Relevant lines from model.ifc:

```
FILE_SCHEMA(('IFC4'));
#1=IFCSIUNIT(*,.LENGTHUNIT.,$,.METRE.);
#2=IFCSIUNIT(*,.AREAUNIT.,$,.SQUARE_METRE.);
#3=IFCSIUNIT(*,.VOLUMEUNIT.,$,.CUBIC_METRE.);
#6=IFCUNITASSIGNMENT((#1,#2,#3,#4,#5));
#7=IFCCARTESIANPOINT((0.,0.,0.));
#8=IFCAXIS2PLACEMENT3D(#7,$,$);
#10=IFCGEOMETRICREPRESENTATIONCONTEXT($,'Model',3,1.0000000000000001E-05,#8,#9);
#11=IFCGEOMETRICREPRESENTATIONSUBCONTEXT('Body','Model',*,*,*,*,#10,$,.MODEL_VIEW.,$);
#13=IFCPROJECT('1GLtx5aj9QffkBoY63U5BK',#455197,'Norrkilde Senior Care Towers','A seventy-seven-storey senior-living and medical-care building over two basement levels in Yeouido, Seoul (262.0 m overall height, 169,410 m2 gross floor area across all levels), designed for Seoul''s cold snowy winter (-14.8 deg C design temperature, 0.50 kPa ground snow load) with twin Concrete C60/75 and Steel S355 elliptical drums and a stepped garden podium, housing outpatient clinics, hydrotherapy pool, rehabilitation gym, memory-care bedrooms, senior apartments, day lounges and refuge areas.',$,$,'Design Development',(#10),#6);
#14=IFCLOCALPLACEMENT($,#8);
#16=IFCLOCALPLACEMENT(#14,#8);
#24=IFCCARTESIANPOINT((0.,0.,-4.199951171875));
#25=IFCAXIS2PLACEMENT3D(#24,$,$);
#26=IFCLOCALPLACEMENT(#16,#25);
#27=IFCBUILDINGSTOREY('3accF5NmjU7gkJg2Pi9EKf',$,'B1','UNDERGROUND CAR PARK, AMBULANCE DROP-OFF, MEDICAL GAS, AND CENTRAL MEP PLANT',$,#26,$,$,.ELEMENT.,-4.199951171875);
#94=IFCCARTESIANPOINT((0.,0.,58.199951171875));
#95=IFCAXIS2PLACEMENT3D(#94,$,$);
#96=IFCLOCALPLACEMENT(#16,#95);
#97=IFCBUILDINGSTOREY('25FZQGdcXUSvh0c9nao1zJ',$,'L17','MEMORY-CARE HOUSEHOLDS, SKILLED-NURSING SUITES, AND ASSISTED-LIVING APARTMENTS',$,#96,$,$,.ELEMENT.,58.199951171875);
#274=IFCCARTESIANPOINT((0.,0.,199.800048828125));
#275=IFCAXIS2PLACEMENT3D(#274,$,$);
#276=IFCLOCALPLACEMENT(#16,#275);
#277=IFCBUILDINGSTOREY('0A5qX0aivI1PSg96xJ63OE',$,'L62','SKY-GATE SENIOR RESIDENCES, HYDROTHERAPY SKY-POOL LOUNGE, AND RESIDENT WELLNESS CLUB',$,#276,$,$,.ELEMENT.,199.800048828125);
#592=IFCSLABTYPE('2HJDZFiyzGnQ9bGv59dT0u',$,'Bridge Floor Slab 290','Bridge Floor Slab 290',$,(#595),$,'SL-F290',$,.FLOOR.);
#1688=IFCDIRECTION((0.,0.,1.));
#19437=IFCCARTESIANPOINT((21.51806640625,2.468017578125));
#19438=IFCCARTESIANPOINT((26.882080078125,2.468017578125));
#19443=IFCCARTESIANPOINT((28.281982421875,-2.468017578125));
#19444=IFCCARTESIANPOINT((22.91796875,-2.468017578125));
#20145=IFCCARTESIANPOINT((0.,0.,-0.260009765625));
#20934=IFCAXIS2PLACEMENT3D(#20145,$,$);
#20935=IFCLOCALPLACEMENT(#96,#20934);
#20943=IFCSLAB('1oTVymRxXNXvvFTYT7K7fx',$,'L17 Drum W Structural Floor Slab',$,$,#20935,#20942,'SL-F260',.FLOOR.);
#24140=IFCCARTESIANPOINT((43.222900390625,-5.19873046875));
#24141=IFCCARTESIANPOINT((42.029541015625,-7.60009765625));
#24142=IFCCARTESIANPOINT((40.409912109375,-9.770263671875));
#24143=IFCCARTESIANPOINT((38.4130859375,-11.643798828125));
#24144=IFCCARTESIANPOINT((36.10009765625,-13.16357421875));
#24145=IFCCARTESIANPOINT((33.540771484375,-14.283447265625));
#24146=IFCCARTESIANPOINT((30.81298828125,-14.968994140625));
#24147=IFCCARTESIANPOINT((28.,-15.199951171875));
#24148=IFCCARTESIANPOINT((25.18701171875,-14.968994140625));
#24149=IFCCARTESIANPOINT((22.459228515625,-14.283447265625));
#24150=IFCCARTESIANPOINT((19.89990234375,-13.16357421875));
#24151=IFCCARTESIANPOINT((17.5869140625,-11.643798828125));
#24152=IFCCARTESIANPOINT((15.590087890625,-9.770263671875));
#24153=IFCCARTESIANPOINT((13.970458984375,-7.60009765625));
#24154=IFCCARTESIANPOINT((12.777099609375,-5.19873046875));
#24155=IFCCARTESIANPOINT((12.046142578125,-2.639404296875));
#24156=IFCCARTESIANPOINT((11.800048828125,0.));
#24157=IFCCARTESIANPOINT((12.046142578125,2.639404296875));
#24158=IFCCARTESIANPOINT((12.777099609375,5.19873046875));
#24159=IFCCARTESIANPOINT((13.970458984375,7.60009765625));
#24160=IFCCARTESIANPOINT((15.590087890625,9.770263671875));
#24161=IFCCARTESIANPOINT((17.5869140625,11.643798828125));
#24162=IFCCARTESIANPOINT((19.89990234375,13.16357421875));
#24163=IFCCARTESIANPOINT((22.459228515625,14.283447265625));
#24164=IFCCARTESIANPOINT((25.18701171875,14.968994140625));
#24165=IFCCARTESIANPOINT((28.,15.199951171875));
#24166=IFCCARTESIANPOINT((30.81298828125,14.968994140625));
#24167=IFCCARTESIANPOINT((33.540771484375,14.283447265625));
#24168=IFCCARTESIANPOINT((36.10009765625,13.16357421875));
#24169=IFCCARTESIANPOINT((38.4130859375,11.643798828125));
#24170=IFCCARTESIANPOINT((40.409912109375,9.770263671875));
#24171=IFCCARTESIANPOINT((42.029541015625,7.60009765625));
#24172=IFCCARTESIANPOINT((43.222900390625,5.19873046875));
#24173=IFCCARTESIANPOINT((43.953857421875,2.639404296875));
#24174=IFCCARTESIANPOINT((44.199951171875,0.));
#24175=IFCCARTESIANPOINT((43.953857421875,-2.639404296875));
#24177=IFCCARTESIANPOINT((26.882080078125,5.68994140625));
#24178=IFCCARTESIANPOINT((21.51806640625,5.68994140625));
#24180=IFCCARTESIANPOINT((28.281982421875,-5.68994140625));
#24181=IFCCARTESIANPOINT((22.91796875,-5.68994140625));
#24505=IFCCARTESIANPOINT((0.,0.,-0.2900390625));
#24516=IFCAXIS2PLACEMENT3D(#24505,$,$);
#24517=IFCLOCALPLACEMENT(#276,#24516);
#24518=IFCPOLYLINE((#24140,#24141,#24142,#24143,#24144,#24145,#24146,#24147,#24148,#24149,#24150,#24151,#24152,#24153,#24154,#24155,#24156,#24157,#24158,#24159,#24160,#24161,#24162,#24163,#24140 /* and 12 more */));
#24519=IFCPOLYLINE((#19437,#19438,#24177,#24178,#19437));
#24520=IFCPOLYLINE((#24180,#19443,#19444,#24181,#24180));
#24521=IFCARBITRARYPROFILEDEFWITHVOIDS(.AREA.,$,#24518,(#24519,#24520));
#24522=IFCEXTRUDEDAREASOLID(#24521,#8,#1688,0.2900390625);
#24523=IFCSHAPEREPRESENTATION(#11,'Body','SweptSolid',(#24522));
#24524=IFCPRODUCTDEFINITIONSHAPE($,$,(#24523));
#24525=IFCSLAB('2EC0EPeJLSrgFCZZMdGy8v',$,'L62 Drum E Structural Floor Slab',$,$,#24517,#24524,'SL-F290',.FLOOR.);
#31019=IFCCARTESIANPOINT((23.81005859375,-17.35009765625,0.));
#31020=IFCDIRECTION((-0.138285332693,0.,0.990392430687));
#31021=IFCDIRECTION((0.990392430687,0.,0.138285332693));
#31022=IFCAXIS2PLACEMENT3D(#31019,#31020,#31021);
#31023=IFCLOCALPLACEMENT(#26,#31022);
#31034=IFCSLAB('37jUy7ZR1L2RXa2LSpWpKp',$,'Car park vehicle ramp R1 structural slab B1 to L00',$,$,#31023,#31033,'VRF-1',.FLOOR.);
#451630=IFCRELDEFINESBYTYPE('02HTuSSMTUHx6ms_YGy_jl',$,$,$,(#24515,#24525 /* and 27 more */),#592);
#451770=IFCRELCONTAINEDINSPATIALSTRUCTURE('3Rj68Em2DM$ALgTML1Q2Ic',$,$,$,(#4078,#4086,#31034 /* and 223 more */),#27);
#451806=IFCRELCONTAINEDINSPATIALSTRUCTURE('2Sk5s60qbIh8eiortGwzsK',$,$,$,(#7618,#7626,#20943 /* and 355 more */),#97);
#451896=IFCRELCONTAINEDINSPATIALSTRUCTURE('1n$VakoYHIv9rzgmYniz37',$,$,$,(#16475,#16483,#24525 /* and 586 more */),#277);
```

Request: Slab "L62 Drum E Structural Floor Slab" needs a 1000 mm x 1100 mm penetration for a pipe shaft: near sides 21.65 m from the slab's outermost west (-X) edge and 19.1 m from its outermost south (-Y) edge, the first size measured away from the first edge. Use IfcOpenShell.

```python
import numpy as np
import ifcopenshell
import ifcopenshell.api.feature
import ifcopenshell.api.geometry
import ifcopenshell.api.root
import ifcopenshell.geom
import ifcopenshell.util.placement
import ifcopenshell.util.representation
import ifcopenshell.util.shape
import ifcopenshell.util.unit

model = ifcopenshell.open("model.ifc")
unit_scale = ifcopenshell.util.unit.calculate_unit_scale(model)
settings = ifcopenshell.geom.settings()


def volume(element):
    """Net volume in cubic metres, openings subtracted."""
    shape = ifcopenshell.geom.create_shape(settings, element)
    return ifcopenshell.util.shape.get_volume(shape.geometry)


slab = model.by_guid("2EC0EPeJLSrgFCZZMdGy8v")
before = volume(slab)

# Extent in the slab's own axes, in metres. The edges named are its -X and -Y sides.
slab_shape = ifcopenshell.geom.create_shape(settings, slab)
vertices = ifcopenshell.util.shape.get_vertices(slab_shape.geometry)
x_min, y_min, bottom = vertices.min(axis=0)
top = vertices[:, 2].max()

opening = ifcopenshell.api.root.create_entity(model, ifc_class="IfcOpeningElement", name="Pipe shaft opening", predefined_type="OPENING")
context = ifcopenshell.util.representation.get_context(model, "Model", "Body", "MODEL_VIEW")
width, depth = 1, 1.1
outline = [(0.0, 0.0), (width, 0.0), (width, depth), (0.0, depth), (0.0, 0.0)]
# Overshoot both faces by 50 mm so the cut is clean.
shape = ifcopenshell.api.geometry.add_slab_representation(
    model, context=context, depth=top - bottom + 0.1, polyline=outline
)
ifcopenshell.api.geometry.assign_representation(model, product=opening, representation=shape)

matrix = ifcopenshell.util.placement.get_local_placement(slab.ObjectPlacement)
matrix[:, 3] = matrix @ np.append(np.array([x_min + 21.65, y_min + 19.1, bottom - 0.05]) / unit_scale, 1.0)
ifcopenshell.api.geometry.edit_object_placement(model, product=opening, matrix=matrix, is_si=False)
ifcopenshell.api.feature.add_feature(model, feature=opening, element=slab)

after = volume(slab)

print(f"slab volume {before:.3f} -> {after:.3f} m3")

model.write("model_v2.ifc")
```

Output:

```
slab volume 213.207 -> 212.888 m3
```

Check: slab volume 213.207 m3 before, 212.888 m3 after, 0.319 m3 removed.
